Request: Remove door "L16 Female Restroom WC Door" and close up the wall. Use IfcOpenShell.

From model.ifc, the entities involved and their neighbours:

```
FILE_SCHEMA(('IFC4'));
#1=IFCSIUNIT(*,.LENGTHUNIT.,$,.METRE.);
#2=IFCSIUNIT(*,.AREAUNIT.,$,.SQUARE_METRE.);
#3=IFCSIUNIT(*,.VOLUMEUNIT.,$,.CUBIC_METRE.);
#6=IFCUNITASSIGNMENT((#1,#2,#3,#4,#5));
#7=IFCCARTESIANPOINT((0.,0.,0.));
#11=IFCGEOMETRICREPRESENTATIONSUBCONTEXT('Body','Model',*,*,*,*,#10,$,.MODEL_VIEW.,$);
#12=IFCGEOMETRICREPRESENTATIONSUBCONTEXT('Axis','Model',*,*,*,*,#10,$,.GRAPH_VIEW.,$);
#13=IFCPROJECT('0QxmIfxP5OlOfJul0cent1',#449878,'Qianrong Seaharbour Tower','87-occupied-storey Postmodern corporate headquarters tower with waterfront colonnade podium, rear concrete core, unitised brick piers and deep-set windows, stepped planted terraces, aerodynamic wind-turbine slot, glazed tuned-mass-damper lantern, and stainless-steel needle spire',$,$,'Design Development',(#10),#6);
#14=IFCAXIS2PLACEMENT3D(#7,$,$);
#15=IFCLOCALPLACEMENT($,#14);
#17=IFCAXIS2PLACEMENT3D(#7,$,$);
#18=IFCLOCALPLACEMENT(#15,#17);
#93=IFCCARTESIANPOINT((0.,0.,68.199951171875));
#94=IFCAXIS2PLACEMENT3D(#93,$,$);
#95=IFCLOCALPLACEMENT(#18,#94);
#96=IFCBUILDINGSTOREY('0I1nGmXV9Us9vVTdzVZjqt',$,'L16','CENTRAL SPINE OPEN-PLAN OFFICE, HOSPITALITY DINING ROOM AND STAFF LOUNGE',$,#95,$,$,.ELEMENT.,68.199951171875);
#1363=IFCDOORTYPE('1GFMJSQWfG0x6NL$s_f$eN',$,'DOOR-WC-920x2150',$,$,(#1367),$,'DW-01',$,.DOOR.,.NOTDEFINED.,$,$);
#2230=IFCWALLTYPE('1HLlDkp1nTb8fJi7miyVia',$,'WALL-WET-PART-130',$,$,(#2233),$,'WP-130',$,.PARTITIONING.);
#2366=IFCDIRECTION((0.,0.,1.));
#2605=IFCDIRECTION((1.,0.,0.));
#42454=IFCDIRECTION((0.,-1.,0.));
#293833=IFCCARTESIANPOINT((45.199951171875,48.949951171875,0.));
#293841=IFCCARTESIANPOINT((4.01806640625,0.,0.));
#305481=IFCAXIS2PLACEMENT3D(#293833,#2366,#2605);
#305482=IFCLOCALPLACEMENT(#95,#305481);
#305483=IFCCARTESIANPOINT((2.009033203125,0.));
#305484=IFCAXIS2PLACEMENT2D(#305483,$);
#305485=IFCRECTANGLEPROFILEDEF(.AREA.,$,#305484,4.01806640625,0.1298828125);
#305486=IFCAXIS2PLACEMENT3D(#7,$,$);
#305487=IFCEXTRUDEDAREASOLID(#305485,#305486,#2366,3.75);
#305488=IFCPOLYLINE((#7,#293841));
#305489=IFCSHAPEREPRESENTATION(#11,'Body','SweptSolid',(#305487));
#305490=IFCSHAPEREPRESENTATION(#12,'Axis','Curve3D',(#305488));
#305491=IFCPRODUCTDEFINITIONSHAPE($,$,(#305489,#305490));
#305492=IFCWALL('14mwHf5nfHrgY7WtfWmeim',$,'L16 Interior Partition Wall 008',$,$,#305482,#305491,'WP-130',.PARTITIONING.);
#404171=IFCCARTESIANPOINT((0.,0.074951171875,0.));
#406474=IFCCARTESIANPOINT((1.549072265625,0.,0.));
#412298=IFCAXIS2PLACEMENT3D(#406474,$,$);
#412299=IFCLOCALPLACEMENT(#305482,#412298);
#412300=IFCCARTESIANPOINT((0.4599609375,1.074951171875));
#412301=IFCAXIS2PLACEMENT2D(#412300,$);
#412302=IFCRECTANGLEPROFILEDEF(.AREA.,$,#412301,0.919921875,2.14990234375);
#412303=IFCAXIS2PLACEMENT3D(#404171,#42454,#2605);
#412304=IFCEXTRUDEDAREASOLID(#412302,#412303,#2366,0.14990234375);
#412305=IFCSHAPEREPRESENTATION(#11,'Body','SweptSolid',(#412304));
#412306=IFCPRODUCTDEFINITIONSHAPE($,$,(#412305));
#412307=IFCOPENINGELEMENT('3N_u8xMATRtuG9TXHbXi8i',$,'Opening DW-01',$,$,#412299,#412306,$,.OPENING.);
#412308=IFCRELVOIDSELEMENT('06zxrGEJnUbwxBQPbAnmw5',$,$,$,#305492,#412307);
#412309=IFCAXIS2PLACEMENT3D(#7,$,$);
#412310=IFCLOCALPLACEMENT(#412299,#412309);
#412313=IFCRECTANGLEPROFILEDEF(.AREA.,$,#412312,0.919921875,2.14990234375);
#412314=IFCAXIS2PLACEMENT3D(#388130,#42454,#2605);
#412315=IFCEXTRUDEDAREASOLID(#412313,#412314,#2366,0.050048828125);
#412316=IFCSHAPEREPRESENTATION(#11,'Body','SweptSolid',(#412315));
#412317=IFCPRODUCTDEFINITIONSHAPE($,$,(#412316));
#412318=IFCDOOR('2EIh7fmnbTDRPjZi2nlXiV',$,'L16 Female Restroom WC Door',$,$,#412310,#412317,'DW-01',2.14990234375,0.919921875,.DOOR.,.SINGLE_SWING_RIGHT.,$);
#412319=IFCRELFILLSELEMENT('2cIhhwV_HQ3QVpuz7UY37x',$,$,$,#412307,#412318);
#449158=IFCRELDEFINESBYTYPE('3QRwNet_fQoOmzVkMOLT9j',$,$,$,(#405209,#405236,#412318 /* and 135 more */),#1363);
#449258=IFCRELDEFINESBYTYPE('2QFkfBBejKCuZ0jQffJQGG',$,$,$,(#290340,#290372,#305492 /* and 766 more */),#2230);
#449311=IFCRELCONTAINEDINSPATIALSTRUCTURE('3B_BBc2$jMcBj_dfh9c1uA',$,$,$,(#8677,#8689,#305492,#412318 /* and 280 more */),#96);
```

```python
import ifcopenshell
import ifcopenshell.api.feature
import ifcopenshell.api.root
import ifcopenshell.geom
import ifcopenshell.util.shape

model = ifcopenshell.open("model.ifc")
settings = ifcopenshell.geom.settings()


def volume(element):
    """Net volume in cubic metres, openings subtracted."""
    shape = ifcopenshell.geom.create_shape(settings, element)
    return ifcopenshell.util.shape.get_volume(shape.geometry)


door = model.by_guid("2EIh7fmnbTDRPjZi2nlXiV")
opening = door.FillsVoids[0].RelatingOpeningElement
wall = opening.VoidsElements[0].RelatingBuildingElement
before = volume(wall)

ifcopenshell.api.root.remove_product(model, product=door)
ifcopenshell.api.feature.remove_feature(model, feature=opening)

after = volume(wall)

print(f"wall volume {before:.3f} -> {after:.3f} m3")

model.write("model_edited.ifc")
```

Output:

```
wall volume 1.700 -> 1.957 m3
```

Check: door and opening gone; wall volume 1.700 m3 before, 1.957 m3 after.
